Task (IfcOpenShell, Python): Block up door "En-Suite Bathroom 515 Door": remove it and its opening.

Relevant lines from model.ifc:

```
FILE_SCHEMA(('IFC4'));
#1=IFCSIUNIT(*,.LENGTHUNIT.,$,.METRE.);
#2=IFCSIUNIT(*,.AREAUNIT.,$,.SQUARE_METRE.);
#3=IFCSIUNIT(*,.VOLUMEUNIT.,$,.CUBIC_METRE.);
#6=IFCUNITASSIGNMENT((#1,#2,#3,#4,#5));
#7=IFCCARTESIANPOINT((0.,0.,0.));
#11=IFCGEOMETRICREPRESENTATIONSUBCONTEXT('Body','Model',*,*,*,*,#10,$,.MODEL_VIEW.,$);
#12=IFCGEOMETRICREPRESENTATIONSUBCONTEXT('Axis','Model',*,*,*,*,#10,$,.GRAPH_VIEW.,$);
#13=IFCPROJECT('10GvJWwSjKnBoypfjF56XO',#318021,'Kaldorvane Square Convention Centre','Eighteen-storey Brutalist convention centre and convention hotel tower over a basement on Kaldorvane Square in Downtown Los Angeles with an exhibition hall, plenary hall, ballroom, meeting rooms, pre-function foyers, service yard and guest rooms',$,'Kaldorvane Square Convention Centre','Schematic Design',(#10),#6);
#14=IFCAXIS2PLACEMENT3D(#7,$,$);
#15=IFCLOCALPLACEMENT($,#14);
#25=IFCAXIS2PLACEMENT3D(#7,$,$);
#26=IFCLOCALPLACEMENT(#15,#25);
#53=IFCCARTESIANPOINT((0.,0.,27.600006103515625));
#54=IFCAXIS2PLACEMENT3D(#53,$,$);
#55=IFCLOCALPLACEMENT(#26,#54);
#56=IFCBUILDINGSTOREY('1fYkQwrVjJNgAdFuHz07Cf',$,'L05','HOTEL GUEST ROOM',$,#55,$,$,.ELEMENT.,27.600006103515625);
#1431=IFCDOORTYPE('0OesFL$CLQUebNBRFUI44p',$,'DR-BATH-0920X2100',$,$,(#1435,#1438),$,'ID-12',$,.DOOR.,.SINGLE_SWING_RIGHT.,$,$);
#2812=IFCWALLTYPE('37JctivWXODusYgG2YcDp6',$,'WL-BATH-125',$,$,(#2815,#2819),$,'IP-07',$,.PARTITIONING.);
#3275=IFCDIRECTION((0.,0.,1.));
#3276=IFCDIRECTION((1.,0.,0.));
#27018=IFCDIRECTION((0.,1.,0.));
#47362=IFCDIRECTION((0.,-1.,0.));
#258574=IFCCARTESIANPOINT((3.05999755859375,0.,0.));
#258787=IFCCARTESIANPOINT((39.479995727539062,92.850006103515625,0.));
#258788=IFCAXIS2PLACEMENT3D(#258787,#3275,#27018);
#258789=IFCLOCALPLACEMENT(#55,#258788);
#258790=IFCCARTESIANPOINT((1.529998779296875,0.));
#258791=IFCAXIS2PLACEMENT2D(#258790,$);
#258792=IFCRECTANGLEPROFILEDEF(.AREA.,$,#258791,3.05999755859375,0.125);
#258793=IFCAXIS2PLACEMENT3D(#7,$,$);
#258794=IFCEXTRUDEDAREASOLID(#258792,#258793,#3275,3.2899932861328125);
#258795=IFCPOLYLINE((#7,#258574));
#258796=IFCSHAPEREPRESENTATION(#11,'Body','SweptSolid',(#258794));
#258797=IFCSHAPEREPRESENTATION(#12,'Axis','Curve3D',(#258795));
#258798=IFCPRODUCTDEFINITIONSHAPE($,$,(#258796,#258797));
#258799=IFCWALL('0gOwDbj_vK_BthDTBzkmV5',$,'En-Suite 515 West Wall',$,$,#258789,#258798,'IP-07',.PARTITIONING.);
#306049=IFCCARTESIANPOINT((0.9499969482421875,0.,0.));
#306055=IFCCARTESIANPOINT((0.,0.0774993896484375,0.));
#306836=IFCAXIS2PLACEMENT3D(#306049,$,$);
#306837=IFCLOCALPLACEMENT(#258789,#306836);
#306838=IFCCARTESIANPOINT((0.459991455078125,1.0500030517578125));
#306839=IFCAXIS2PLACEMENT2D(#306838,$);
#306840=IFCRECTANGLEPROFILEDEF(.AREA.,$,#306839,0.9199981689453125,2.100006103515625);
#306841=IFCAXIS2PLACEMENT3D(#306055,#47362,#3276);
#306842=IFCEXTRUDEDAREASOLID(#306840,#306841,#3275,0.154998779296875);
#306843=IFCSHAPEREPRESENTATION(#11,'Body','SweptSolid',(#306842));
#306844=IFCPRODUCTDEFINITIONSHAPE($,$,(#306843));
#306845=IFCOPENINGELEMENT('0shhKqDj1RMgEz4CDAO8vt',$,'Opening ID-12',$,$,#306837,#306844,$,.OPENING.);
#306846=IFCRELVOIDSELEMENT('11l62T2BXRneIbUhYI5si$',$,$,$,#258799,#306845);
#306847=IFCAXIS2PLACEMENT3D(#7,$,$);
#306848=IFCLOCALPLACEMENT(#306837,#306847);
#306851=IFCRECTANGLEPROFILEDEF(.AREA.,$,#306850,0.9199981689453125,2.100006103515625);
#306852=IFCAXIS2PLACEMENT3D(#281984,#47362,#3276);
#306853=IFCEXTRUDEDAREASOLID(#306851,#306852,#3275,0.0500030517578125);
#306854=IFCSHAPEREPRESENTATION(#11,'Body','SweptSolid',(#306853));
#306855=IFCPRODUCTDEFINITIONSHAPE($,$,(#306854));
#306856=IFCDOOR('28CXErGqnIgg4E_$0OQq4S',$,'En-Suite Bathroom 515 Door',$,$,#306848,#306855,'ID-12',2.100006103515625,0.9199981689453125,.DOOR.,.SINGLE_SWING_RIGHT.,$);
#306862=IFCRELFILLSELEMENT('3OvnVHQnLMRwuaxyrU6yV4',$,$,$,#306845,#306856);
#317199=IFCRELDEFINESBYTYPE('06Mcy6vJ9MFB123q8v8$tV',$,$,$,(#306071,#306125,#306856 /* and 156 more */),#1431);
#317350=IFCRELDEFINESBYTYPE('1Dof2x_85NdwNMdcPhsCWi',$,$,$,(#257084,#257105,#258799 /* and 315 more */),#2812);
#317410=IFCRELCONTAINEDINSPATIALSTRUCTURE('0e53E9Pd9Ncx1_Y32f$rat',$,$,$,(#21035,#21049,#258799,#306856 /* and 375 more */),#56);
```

```python
import ifcopenshell
import ifcopenshell.api.feature
import ifcopenshell.api.root
import ifcopenshell.geom
import ifcopenshell.util.shape

model = ifcopenshell.open("model.ifc")
settings = ifcopenshell.geom.settings()


def volume(element):
    """Net volume in cubic metres, openings subtracted."""
    shape = ifcopenshell.geom.create_shape(settings, element)
    return ifcopenshell.util.shape.get_volume(shape.geometry)


door = model.by_guid("28CXErGqnIgg4E_$0OQq4S")
opening = door.FillsVoids[0].RelatingOpeningElement
wall = opening.VoidsElements[0].RelatingBuildingElement
before = volume(wall)

ifcopenshell.api.root.remove_product(model, product=door)
ifcopenshell.api.feature.remove_feature(model, feature=opening)

after = volume(wall)

print(f"wall volume {before:.3f} -> {after:.3f} m3")

model.write("model_rev.ifc")
```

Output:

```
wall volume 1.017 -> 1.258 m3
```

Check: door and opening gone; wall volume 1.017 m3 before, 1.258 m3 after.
